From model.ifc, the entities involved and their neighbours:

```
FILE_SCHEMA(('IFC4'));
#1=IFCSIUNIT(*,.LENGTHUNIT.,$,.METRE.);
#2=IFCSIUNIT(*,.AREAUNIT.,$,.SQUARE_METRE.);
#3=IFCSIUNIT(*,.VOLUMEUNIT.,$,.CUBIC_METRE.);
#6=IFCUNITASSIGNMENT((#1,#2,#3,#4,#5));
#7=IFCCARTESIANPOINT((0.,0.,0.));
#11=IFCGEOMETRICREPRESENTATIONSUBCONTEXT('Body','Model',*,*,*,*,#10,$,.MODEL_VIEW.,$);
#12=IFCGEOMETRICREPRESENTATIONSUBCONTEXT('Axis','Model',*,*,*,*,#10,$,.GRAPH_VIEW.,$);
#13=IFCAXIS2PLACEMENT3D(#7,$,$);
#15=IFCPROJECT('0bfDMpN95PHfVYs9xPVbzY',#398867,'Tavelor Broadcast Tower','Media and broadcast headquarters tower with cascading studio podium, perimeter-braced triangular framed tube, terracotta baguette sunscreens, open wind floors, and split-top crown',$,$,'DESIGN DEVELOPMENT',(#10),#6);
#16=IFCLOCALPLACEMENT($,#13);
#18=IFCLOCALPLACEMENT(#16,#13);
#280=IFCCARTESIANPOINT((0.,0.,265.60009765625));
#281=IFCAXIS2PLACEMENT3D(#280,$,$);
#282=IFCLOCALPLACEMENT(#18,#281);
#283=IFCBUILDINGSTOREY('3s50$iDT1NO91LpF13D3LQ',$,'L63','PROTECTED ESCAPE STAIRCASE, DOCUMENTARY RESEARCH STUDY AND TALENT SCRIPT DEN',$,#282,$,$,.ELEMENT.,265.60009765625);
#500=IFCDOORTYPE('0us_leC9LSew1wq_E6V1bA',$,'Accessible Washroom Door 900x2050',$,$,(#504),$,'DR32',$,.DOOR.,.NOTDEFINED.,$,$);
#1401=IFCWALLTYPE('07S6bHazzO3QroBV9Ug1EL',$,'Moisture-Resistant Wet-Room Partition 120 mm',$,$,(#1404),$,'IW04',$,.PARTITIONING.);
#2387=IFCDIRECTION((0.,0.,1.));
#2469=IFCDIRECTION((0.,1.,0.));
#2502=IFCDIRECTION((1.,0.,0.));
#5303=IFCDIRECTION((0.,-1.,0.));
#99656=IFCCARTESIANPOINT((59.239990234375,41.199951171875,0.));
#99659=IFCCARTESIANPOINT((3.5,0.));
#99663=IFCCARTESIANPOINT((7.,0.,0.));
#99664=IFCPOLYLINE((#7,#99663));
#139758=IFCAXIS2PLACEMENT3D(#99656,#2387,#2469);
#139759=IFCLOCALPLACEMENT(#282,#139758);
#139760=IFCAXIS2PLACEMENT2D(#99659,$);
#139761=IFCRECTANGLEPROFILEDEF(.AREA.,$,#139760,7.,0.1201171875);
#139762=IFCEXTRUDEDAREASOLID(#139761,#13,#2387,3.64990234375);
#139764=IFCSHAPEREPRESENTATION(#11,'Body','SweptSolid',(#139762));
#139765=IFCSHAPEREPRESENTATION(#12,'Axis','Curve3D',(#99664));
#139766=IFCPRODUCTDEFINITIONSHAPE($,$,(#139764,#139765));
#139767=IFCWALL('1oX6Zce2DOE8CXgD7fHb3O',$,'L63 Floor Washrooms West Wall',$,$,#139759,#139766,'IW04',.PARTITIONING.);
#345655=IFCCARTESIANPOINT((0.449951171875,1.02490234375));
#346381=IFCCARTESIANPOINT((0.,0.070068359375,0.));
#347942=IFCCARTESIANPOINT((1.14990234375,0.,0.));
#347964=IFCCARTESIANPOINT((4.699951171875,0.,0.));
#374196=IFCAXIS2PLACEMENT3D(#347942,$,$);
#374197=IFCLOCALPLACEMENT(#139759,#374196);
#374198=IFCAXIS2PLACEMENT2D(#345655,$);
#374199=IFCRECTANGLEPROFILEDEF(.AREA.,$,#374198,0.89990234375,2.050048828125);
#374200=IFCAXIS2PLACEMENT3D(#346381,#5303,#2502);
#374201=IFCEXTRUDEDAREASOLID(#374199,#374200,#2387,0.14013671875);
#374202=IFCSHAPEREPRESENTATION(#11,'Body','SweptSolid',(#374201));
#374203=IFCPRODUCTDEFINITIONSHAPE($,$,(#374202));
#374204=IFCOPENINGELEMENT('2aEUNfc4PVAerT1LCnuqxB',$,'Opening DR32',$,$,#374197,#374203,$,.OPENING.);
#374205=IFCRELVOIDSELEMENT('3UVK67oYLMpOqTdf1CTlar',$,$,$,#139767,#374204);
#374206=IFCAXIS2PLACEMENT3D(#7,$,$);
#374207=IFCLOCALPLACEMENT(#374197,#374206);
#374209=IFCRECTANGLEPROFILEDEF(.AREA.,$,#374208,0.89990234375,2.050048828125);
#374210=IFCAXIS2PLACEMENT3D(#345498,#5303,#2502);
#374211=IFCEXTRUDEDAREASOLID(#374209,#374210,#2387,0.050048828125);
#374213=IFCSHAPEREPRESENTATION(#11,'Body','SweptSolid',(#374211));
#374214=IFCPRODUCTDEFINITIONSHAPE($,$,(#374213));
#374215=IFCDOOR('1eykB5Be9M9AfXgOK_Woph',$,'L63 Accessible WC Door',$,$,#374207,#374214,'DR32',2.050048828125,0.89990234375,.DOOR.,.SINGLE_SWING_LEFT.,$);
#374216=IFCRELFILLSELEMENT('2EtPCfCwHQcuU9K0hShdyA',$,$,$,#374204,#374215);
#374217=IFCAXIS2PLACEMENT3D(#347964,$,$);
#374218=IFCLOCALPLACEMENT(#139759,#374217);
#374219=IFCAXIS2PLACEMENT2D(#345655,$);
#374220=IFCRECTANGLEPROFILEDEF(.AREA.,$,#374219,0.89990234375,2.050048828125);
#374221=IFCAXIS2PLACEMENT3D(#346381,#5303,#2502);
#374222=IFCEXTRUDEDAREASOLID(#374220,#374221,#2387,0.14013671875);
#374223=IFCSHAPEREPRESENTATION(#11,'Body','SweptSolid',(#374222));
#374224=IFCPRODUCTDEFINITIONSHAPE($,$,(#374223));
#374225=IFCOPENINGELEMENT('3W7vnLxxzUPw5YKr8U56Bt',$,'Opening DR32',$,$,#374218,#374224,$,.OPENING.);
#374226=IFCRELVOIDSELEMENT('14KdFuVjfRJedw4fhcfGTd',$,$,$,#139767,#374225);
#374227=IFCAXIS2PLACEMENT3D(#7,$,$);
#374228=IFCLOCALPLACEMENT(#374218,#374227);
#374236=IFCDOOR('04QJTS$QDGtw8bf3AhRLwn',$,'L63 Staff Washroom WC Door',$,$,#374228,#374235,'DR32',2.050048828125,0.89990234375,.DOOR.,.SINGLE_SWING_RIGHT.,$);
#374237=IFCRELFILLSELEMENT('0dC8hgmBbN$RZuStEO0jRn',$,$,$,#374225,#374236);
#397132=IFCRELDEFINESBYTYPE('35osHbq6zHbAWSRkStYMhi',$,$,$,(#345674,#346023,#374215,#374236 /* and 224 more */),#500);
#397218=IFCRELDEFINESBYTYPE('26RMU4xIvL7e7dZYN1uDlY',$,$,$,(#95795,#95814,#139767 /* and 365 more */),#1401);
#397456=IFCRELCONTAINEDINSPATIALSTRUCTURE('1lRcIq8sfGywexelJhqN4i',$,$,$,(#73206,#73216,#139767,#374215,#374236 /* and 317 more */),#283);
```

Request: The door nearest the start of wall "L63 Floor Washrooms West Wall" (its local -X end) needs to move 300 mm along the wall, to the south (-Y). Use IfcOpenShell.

```python
import ifcopenshell
import ifcopenshell.api.geometry
import ifcopenshell.util.placement

model = ifcopenshell.open("model.ifc")

door = model.by_id(374215)
opening = door.FillsVoids[0].RelatingOpeningElement
wall = opening.VoidsElements[0].RelatingBuildingElement

wall_matrix = ifcopenshell.util.placement.get_local_placement(wall.ObjectPlacement)
shift = wall_matrix[:3, 0] * -0.3
before = ifcopenshell.util.placement.get_local_placement(door.ObjectPlacement)[:3, 3].copy()

# The door is placed relative to its opening, so it follows when the opening moves.
matrix = ifcopenshell.util.placement.get_local_placement(opening.ObjectPlacement)
matrix[:3, 3] += shift
ifcopenshell.api.geometry.edit_object_placement(
    model, product=opening, matrix=matrix, is_si=False, should_transform_children=True
)

after = ifcopenshell.util.placement.get_local_placement(door.ObjectPlacement)[:3, 3]
print("door moved by", (after - before).round(3) + 0.0)

model.write("model_rev.ifc")
```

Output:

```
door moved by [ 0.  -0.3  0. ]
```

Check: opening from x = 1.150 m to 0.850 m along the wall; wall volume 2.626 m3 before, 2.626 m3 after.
